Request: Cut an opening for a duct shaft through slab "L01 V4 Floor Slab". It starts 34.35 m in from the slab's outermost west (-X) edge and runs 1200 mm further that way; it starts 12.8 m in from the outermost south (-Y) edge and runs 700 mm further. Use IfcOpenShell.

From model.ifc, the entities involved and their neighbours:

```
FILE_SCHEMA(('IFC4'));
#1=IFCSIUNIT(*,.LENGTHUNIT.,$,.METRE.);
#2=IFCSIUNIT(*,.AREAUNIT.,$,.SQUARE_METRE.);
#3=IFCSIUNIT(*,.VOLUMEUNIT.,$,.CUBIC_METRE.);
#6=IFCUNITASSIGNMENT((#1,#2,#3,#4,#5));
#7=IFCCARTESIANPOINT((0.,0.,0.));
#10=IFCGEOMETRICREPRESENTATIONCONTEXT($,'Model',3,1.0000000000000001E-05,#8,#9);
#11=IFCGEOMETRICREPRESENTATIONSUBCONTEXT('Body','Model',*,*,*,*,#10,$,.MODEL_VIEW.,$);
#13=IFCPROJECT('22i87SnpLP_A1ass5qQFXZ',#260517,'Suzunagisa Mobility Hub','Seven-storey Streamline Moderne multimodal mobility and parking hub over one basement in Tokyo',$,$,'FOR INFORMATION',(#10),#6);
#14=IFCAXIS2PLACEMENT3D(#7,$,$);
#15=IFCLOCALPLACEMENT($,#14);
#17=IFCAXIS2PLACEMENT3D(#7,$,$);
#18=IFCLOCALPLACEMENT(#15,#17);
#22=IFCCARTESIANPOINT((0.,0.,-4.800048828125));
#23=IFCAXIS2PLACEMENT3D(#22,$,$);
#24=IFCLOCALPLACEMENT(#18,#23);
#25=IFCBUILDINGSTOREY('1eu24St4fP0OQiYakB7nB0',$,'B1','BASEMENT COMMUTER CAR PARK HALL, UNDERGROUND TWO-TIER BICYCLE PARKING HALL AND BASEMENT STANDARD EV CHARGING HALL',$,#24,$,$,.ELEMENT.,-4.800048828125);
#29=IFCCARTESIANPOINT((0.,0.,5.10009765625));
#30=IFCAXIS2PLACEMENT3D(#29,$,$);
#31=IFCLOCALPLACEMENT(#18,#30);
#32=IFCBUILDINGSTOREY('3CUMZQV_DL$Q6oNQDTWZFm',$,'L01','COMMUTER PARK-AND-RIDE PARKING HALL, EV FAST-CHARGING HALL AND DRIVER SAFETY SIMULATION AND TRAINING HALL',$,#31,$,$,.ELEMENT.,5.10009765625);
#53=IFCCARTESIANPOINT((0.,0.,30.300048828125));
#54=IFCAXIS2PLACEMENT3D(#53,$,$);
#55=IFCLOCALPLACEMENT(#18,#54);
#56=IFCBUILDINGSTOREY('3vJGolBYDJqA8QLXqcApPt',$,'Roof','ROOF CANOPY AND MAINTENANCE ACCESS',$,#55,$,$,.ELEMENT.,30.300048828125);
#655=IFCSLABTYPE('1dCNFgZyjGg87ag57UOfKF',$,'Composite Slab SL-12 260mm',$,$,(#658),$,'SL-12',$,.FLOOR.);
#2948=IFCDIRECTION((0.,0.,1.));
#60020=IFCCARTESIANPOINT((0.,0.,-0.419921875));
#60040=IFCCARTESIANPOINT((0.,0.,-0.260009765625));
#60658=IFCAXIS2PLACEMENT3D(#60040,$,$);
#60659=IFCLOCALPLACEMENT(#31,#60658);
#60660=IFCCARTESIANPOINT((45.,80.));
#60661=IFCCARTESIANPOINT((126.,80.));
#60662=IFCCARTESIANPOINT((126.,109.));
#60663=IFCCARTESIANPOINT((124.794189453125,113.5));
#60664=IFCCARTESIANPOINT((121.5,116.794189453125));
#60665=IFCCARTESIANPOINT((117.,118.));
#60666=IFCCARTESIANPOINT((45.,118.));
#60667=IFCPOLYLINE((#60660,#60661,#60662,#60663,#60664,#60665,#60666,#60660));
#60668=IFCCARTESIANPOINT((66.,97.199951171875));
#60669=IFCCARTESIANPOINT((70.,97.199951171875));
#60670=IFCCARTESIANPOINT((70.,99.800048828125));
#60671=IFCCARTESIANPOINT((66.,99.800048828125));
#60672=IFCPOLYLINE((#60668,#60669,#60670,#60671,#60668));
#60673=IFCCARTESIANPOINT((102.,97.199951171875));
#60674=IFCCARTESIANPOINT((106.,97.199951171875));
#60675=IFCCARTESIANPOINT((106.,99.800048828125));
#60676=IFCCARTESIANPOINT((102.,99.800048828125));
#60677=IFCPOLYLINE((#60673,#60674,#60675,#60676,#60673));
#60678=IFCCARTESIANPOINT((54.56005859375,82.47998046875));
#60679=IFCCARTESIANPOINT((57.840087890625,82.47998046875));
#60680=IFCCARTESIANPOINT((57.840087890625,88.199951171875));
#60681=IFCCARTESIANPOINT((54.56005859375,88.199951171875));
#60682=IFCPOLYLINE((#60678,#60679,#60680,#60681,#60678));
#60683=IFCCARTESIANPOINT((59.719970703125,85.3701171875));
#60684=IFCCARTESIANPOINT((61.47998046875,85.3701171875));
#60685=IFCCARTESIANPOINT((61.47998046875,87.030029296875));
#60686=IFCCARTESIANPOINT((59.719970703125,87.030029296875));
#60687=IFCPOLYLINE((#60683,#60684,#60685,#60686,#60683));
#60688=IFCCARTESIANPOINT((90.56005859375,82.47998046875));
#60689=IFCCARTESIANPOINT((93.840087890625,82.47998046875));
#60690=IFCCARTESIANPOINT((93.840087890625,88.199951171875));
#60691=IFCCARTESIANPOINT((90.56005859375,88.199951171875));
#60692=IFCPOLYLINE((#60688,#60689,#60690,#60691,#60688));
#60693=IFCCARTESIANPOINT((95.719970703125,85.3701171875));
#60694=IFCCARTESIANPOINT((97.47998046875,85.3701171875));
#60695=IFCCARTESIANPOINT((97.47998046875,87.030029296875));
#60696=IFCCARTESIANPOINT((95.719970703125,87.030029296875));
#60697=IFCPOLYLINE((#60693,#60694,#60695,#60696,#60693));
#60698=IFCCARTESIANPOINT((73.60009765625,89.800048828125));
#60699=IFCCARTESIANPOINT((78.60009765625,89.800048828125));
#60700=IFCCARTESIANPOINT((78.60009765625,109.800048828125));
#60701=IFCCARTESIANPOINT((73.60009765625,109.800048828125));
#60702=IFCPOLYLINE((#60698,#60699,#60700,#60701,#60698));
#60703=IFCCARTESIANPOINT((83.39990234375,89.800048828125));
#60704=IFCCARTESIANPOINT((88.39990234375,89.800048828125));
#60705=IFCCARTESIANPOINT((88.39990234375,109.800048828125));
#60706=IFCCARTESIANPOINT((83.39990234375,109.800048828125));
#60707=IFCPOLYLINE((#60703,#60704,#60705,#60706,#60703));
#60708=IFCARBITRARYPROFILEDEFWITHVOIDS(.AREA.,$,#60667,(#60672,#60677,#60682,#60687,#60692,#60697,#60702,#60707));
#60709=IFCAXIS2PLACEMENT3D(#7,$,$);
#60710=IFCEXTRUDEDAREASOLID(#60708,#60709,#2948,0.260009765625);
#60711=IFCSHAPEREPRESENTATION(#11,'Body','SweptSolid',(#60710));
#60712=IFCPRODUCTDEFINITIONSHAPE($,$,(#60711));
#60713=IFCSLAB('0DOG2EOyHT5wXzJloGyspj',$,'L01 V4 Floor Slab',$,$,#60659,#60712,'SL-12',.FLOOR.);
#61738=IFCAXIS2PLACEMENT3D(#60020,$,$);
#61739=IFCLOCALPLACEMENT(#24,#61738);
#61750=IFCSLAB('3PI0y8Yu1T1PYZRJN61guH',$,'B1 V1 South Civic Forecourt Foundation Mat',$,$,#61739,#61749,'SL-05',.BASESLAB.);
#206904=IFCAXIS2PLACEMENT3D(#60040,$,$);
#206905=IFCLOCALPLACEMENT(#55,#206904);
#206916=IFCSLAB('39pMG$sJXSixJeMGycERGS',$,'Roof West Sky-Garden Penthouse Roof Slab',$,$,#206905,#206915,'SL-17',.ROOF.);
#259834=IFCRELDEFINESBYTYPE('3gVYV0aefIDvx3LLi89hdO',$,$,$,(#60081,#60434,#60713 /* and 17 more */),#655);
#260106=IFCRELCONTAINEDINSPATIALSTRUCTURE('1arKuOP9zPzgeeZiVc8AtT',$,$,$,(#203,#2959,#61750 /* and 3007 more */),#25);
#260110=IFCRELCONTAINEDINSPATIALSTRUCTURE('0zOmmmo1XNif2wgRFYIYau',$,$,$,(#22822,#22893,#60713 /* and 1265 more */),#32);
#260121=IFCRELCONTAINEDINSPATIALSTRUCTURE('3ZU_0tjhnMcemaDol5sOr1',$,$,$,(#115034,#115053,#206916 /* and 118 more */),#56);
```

```python
import numpy as np
import ifcopenshell
import ifcopenshell.api.feature
import ifcopenshell.api.geometry
import ifcopenshell.api.root
import ifcopenshell.geom
import ifcopenshell.util.placement
import ifcopenshell.util.representation
import ifcopenshell.util.shape
import ifcopenshell.util.unit

model = ifcopenshell.open("model.ifc")
unit_scale = ifcopenshell.util.unit.calculate_unit_scale(model)
settings = ifcopenshell.geom.settings()


def volume(element):
    """Net volume in cubic metres, openings subtracted."""
    shape = ifcopenshell.geom.create_shape(settings, element)
    return ifcopenshell.util.shape.get_volume(shape.geometry)


slab = model.by_id(60713)
before = volume(slab)

# Extent in the slab's own axes, in metres. The edges named are its -X and -Y sides.
slab_shape = ifcopenshell.geom.create_shape(settings, slab)
vertices = ifcopenshell.util.shape.get_vertices(slab_shape.geometry)
x_min, y_min, bottom = vertices.min(axis=0)
top = vertices[:, 2].max()

opening = ifcopenshell.api.root.create_entity(model, ifc_class="IfcOpeningElement", name="Duct shaft opening", predefined_type="OPENING")
context = ifcopenshell.util.representation.get_context(model, "Model", "Body", "MODEL_VIEW")
width, depth = 1.2, 0.7
outline = [(0.0, 0.0), (width, 0.0), (width, depth), (0.0, depth), (0.0, 0.0)]
# Overshoot both faces by 50 mm so the cut is clean.
shape = ifcopenshell.api.geometry.add_slab_representation(
    model, context=context, depth=top - bottom + 0.1, polyline=outline
)
ifcopenshell.api.geometry.assign_representation(model, product=opening, representation=shape)

matrix = ifcopenshell.util.placement.get_local_placement(slab.ObjectPlacement)
matrix[:, 3] = matrix @ np.append(np.array([x_min + 34.35, y_min + 12.8, bottom - 0.05]) / unit_scale, 1.0)
ifcopenshell.api.geometry.edit_object_placement(model, product=opening, matrix=matrix, is_si=False)
ifcopenshell.api.feature.add_feature(model, feature=opening, element=slab)

after = volume(slab)

print(f"slab volume {before:.3f} -> {after:.3f} m3")

model.write("model_rev.ifc")
```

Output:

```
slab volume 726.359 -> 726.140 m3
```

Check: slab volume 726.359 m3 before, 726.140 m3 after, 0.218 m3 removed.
